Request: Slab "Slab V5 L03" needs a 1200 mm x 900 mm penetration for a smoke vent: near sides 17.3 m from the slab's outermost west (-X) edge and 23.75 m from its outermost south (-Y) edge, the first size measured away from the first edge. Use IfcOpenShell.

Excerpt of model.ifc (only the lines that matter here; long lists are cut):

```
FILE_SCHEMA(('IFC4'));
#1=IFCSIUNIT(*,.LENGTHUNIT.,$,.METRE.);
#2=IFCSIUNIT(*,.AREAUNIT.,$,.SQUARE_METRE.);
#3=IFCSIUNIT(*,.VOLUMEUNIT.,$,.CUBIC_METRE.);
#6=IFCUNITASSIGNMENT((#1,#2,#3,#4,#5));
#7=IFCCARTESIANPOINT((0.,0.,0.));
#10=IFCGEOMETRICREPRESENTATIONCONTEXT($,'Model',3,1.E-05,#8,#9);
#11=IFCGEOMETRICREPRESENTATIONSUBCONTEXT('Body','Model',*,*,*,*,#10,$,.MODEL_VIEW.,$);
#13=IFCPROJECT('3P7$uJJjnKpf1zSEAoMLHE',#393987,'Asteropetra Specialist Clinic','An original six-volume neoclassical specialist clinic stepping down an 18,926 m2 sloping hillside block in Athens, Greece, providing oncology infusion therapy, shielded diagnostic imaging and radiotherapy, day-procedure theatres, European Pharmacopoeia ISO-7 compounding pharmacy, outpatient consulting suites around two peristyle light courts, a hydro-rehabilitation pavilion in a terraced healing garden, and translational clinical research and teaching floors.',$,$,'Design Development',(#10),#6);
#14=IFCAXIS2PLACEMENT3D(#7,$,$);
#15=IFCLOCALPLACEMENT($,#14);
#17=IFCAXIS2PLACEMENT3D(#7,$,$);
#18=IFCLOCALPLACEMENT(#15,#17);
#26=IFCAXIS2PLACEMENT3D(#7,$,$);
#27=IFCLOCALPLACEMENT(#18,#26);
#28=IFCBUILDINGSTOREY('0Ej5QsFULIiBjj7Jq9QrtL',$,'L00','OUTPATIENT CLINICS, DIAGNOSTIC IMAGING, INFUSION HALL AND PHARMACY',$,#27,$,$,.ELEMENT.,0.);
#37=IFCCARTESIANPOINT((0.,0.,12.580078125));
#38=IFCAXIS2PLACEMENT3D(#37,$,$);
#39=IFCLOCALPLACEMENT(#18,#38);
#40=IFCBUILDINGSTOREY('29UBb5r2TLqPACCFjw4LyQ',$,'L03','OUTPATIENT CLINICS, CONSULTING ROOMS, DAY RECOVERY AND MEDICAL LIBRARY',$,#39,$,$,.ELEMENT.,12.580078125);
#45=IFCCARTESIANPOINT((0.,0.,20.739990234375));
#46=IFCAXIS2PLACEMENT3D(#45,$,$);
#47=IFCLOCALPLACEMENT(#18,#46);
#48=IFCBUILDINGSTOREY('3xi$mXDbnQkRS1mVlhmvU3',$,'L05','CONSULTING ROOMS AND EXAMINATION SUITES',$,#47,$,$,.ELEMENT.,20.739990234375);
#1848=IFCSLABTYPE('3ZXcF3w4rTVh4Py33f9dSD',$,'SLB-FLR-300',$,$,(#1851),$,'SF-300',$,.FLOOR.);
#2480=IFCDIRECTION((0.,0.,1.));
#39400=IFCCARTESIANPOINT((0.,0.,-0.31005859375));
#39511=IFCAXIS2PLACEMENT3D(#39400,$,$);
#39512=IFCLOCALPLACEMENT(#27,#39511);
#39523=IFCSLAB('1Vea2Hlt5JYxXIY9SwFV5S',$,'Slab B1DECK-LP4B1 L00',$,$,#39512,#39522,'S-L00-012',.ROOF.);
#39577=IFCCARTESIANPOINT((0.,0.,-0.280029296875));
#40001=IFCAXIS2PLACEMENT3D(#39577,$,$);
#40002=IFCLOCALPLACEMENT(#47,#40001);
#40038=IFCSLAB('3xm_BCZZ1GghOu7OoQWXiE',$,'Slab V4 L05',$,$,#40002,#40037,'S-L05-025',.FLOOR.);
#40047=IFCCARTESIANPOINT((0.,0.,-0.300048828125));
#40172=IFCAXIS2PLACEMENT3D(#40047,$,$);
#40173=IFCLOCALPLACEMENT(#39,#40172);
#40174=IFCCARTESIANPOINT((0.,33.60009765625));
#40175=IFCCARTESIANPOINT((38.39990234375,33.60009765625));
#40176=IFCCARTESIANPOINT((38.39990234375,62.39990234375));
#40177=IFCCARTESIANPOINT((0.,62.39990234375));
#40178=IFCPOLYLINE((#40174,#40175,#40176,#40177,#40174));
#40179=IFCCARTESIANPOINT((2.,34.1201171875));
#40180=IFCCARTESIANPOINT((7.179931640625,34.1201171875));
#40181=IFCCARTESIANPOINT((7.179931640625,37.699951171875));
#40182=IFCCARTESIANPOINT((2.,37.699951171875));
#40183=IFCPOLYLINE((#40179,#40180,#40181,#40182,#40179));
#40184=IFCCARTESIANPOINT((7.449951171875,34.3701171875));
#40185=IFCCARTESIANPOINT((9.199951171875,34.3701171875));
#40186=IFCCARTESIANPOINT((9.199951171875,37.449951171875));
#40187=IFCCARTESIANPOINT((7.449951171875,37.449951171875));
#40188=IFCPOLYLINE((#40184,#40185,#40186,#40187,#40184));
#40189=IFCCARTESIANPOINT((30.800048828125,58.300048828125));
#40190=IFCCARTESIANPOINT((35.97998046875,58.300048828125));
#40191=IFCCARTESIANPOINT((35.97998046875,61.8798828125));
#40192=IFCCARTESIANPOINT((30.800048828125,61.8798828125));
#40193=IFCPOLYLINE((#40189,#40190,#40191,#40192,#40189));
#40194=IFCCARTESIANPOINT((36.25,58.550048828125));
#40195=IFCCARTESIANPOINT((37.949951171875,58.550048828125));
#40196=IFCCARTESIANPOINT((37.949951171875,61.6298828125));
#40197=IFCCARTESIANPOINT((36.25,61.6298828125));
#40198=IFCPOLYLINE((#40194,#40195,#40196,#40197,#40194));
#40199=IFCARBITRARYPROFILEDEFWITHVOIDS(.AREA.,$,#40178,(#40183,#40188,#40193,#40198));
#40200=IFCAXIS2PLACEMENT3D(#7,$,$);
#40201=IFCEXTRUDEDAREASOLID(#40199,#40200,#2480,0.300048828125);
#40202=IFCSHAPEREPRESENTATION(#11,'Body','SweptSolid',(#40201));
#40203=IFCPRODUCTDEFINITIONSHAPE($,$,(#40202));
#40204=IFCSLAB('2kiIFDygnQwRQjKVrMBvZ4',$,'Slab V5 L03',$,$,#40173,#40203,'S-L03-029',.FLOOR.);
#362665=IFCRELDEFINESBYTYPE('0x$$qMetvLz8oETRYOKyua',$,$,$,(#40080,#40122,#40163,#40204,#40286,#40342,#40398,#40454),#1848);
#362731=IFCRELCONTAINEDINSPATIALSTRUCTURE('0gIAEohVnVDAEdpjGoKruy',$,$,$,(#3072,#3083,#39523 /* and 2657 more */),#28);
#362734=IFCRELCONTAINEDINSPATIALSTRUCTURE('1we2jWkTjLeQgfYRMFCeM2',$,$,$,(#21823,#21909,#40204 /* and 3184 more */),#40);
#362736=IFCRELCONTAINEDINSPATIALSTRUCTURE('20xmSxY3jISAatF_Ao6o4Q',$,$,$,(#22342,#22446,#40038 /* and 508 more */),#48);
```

```python
import numpy as np
import ifcopenshell
import ifcopenshell.api.feature
import ifcopenshell.api.geometry
import ifcopenshell.api.root
import ifcopenshell.geom
import ifcopenshell.util.placement
import ifcopenshell.util.representation
import ifcopenshell.util.shape
import ifcopenshell.util.unit

model = ifcopenshell.open("model.ifc")
unit_scale = ifcopenshell.util.unit.calculate_unit_scale(model)
settings = ifcopenshell.geom.settings()


def volume(element):
    """Net volume in cubic metres, openings subtracted."""
    shape = ifcopenshell.geom.create_shape(settings, element)
    return ifcopenshell.util.shape.get_volume(shape.geometry)


slab = model.by_id(40204)
before = volume(slab)

# Extent in the slab's own axes, in metres. The edges named are its -X and -Y sides.
slab_shape = ifcopenshell.geom.create_shape(settings, slab)
vertices = ifcopenshell.util.shape.get_vertices(slab_shape.geometry)
x_min, y_min, bottom = vertices.min(axis=0)
top = vertices[:, 2].max()

opening = ifcopenshell.api.root.create_entity(model, ifc_class="IfcOpeningElement", name="Smoke vent opening", predefined_type="OPENING")
context = ifcopenshell.util.representation.get_context(model, "Model", "Body", "MODEL_VIEW")
width, depth = 1.2, 0.9
outline = [(0.0, 0.0), (width, 0.0), (width, depth), (0.0, depth), (0.0, 0.0)]
# Overshoot both faces by 50 mm so the cut is clean.
shape = ifcopenshell.api.geometry.add_slab_representation(
    model, context=context, depth=top - bottom + 0.1, polyline=outline
)
ifcopenshell.api.geometry.assign_representation(model, product=opening, representation=shape)

matrix = ifcopenshell.util.placement.get_local_placement(slab.ObjectPlacement)
matrix[:, 3] = matrix @ np.append(np.array([x_min + 17.3, y_min + 23.75, bottom - 0.05]) / unit_scale, 1.0)
ifcopenshell.api.geometry.edit_object_placement(model, product=opening, matrix=matrix, is_si=False)
ifcopenshell.api.feature.add_feature(model, feature=opening, element=slab)

after = volume(slab)

print(f"slab volume {before:.3f} -> {after:.3f} m3")

model.write("model_updated.ifc")
```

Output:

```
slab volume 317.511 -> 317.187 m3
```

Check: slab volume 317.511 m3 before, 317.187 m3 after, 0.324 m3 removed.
